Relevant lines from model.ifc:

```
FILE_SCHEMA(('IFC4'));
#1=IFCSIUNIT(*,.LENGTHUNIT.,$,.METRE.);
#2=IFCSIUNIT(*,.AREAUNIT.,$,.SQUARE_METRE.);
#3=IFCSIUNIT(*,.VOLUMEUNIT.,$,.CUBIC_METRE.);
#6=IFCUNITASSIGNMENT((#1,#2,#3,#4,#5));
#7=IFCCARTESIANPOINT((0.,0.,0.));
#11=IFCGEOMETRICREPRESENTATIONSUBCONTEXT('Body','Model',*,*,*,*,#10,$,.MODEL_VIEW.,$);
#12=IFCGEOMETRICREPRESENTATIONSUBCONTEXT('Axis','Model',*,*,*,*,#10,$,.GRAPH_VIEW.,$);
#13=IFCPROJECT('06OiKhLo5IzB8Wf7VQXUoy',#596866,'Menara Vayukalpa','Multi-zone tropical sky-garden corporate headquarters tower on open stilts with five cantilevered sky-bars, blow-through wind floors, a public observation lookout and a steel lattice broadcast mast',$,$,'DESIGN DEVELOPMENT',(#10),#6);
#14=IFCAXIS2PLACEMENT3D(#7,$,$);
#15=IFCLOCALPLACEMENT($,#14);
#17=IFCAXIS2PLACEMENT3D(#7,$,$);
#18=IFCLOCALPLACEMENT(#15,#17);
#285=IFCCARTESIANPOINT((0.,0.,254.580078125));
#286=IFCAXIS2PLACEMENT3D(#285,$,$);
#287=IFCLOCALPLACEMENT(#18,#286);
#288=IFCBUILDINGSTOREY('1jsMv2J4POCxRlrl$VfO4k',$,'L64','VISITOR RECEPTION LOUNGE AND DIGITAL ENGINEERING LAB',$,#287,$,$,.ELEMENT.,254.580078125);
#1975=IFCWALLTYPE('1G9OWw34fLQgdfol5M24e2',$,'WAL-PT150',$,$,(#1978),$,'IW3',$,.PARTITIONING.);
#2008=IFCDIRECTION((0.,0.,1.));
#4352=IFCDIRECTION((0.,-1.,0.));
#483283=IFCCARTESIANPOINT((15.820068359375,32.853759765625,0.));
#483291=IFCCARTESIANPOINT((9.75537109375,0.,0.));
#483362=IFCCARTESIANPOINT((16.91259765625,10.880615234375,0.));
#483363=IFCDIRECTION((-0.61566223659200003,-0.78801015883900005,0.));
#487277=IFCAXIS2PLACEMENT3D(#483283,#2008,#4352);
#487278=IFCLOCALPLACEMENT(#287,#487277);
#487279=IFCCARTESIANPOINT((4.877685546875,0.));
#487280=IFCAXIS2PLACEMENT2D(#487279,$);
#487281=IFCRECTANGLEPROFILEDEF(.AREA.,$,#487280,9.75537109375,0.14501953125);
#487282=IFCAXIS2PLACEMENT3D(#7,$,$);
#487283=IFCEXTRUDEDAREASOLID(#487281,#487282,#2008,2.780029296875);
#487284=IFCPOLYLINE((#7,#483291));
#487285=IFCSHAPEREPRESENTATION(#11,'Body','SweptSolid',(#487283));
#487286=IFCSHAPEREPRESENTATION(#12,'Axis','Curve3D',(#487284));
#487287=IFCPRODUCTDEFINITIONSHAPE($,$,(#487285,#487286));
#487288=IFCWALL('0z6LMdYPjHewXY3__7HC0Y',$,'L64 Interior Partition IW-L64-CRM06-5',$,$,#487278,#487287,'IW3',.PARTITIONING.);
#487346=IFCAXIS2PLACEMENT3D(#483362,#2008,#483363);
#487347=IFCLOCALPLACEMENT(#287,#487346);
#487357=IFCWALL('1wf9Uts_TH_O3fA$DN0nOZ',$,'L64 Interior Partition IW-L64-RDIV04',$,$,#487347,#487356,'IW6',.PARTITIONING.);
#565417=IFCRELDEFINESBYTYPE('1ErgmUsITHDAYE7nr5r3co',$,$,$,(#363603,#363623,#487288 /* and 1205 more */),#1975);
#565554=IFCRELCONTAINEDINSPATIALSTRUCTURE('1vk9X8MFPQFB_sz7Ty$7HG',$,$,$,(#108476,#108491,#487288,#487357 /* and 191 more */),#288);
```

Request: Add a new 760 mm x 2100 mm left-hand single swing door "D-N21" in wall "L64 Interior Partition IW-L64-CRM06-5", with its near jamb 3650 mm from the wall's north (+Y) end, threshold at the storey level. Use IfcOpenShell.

```python
import numpy as np
import ifcopenshell
import ifcopenshell.api.feature
import ifcopenshell.api.geometry
import ifcopenshell.api.root
import ifcopenshell.api.spatial
import ifcopenshell.geom
import ifcopenshell.util.element
import ifcopenshell.util.placement
import ifcopenshell.util.representation
import ifcopenshell.util.shape
import ifcopenshell.util.unit

model = ifcopenshell.open("model.ifc")
unit_scale = ifcopenshell.util.unit.calculate_unit_scale(model)
settings = ifcopenshell.geom.settings()


def volume(element):
    """Net volume in cubic metres, openings subtracted."""
    shape = ifcopenshell.geom.create_shape(settings, element)
    return ifcopenshell.util.shape.get_volume(shape.geometry)


wall = model.by_guid("0z6LMdYPjHewXY3__7HC0Y")
storey = ifcopenshell.util.element.get_container(wall, ifc_class="IfcBuildingStorey")
context = ifcopenshell.util.representation.get_context(model, "Model", "Body", "MODEL_VIEW")
before = volume(wall)

width, height, from_end, sill = 0.76, 2.1, 3.65, 0.0  # metres

# The wall runs along its own X axis, and the end named is its -X end.
wall_shape = ifcopenshell.geom.create_shape(settings, wall)
x, y, z = ifcopenshell.util.shape.get_vertices(wall_shape.geometry).T
start = x.min() + from_end
face, thickness = float(y.min()), float(y.max() - y.min())
wall_matrix = ifcopenshell.util.placement.get_local_placement(wall.ObjectPlacement)
level = ifcopenshell.util.placement.get_local_placement(storey.ObjectPlacement)[2, 3]


def in_wall(x, y):
    """Placement at x, y metres in the wall's axes, at sill height."""
    matrix = wall_matrix.copy()
    matrix[:, 3] = wall_matrix @ np.array([x / unit_scale, y / unit_scale, 0.0, 1.0])
    matrix[2, 3] = level + sill / unit_scale
    return matrix


# Opening: a box that overshoots both wall faces by 50 mm.
opening = ifcopenshell.api.root.create_entity(model, ifc_class="IfcOpeningElement", predefined_type="OPENING")
box = ifcopenshell.api.geometry.add_wall_representation(
    model, context=context, length=width, height=height, thickness=thickness + 0.1
)
ifcopenshell.api.geometry.assign_representation(model, product=opening, representation=box)
ifcopenshell.api.geometry.edit_object_placement(model, product=opening, matrix=in_wall(start, face - 0.05), is_si=False)
ifcopenshell.api.feature.add_feature(model, feature=opening, element=wall)

door = ifcopenshell.api.root.create_entity(model, ifc_class="IfcDoor", name="D-N21", predefined_type="DOOR")
door.OverallWidth, door.OverallHeight = width / unit_scale, height / unit_scale
door.OperationType = "SINGLE_SWING_LEFT"
body = ifcopenshell.api.geometry.add_door_representation(
    model,
    context=context,
    overall_width=door.OverallWidth,
    overall_height=door.OverallHeight,
    operation_type="SINGLE_SWING_LEFT",
    lining_properties={"LiningDepth": thickness / unit_scale, "ThresholdDepth": thickness / unit_scale},
)
ifcopenshell.api.geometry.assign_representation(model, product=door, representation=body)
ifcopenshell.api.spatial.assign_container(model, products=[door], relating_structure=storey)
ifcopenshell.api.feature.add_filling(model, opening=opening, element=door)

# The lining spans the wall, so the door starts at the wall face.
ifcopenshell.api.geometry.edit_object_placement(model, product=door, matrix=in_wall(start, face), is_si=False)

after = volume(wall)

print(f"wall volume {before:.3f} -> {after:.3f} m3")

model.write("model_v2.ifc")
```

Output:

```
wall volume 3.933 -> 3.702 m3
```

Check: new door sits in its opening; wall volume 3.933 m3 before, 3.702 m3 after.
